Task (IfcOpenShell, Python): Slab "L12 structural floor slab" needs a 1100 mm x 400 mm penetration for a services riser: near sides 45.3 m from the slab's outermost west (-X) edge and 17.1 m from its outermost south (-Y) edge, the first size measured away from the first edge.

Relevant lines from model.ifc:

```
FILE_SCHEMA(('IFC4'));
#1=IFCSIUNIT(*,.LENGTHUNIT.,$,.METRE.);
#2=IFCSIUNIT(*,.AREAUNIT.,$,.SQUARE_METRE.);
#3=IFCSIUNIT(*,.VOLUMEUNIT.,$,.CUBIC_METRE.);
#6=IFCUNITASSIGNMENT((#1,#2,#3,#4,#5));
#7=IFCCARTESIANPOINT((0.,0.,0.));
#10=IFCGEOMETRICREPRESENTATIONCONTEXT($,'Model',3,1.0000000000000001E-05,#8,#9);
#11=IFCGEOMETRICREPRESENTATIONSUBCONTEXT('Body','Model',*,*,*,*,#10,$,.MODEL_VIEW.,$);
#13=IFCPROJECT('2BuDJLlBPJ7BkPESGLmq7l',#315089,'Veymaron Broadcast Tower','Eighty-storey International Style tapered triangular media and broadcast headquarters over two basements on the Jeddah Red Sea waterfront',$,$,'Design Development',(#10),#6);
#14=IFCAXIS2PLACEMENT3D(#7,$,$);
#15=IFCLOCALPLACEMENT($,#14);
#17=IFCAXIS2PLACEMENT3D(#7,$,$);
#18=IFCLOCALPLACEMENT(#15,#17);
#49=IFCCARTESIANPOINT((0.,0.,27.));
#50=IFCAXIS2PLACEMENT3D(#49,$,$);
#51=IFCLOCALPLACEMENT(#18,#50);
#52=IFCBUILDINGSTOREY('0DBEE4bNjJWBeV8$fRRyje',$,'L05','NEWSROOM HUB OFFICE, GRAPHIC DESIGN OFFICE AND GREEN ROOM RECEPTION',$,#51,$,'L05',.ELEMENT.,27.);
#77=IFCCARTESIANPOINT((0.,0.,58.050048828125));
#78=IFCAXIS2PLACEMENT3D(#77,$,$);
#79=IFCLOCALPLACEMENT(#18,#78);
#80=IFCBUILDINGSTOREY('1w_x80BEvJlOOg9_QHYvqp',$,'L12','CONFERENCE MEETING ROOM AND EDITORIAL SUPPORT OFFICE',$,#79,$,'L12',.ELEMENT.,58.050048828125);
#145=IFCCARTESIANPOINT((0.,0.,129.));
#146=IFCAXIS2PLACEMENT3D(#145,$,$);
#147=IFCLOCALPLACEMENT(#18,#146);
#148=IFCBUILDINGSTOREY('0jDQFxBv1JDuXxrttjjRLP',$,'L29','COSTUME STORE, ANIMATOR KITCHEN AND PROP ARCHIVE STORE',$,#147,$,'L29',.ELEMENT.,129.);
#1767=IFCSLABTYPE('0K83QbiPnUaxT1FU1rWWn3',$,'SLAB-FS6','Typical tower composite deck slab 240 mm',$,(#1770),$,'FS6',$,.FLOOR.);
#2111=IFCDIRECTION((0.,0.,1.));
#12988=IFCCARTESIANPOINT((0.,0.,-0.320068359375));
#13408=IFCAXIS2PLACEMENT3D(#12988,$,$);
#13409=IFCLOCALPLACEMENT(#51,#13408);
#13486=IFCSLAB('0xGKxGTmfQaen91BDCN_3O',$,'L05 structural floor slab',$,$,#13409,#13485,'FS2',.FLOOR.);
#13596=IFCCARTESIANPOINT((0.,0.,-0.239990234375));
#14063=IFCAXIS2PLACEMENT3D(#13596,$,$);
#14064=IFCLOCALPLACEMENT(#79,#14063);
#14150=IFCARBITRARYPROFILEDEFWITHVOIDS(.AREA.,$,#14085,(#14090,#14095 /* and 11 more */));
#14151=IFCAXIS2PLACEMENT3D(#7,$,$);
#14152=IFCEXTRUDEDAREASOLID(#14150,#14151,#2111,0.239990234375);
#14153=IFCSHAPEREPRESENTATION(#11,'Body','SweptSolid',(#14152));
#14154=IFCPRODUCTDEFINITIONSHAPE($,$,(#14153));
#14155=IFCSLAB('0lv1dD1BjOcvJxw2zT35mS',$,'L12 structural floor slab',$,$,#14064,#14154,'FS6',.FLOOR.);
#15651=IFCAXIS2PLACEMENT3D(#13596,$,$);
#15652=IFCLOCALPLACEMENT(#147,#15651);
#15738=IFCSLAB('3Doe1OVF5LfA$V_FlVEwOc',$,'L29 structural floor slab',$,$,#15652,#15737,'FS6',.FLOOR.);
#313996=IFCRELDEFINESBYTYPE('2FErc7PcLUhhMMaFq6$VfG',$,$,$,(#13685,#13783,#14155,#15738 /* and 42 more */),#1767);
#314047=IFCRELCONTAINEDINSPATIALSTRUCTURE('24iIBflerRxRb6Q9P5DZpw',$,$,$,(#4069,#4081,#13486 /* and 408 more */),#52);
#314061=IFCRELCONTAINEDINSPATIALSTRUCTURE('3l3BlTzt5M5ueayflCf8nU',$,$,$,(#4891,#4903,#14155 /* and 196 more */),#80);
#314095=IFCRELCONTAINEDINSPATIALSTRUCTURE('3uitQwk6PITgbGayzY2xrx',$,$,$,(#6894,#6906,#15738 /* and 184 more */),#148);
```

```python
import numpy as np
import ifcopenshell
import ifcopenshell.api.feature
import ifcopenshell.api.geometry
import ifcopenshell.api.root
import ifcopenshell.geom
import ifcopenshell.util.placement
import ifcopenshell.util.representation
import ifcopenshell.util.shape
import ifcopenshell.util.unit

model = ifcopenshell.open("model.ifc")
unit_scale = ifcopenshell.util.unit.calculate_unit_scale(model)
settings = ifcopenshell.geom.settings()


def volume(element):
    """Net volume in cubic metres, openings subtracted."""
    shape = ifcopenshell.geom.create_shape(settings, element)
    return ifcopenshell.util.shape.get_volume(shape.geometry)


slab = model.by_guid("0lv1dD1BjOcvJxw2zT35mS")
before = volume(slab)

# Extent in the slab's own axes, in metres. The edges named are its -X and -Y sides.
slab_shape = ifcopenshell.geom.create_shape(settings, slab)
vertices = ifcopenshell.util.shape.get_vertices(slab_shape.geometry)
x_min, y_min, bottom = vertices.min(axis=0)
top = vertices[:, 2].max()

opening = ifcopenshell.api.root.create_entity(model, ifc_class="IfcOpeningElement", name="Services riser opening", predefined_type="OPENING")
context = ifcopenshell.util.representation.get_context(model, "Model", "Body", "MODEL_VIEW")
width, depth = 1.1, 0.4
outline = [(0.0, 0.0), (width, 0.0), (width, depth), (0.0, depth), (0.0, 0.0)]
# Overshoot both faces by 50 mm so the cut is clean.
shape = ifcopenshell.api.geometry.add_slab_representation(
    model, context=context, depth=top - bottom + 0.1, polyline=outline
)
ifcopenshell.api.geometry.assign_representation(model, product=opening, representation=shape)

matrix = ifcopenshell.util.placement.get_local_placement(slab.ObjectPlacement)
matrix[:, 3] = matrix @ np.append(np.array([x_min + 45.3, y_min + 17.1, bottom - 0.05]) / unit_scale, 1.0)
ifcopenshell.api.geometry.edit_object_placement(model, product=opening, matrix=matrix, is_si=False)
ifcopenshell.api.feature.add_feature(model, feature=opening, element=slab)

after = volume(slab)

print(f"slab volume {before:.3f} -> {after:.3f} m3")

model.write("model_v2.ifc")
```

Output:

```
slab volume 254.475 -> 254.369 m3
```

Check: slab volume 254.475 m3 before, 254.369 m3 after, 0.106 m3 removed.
